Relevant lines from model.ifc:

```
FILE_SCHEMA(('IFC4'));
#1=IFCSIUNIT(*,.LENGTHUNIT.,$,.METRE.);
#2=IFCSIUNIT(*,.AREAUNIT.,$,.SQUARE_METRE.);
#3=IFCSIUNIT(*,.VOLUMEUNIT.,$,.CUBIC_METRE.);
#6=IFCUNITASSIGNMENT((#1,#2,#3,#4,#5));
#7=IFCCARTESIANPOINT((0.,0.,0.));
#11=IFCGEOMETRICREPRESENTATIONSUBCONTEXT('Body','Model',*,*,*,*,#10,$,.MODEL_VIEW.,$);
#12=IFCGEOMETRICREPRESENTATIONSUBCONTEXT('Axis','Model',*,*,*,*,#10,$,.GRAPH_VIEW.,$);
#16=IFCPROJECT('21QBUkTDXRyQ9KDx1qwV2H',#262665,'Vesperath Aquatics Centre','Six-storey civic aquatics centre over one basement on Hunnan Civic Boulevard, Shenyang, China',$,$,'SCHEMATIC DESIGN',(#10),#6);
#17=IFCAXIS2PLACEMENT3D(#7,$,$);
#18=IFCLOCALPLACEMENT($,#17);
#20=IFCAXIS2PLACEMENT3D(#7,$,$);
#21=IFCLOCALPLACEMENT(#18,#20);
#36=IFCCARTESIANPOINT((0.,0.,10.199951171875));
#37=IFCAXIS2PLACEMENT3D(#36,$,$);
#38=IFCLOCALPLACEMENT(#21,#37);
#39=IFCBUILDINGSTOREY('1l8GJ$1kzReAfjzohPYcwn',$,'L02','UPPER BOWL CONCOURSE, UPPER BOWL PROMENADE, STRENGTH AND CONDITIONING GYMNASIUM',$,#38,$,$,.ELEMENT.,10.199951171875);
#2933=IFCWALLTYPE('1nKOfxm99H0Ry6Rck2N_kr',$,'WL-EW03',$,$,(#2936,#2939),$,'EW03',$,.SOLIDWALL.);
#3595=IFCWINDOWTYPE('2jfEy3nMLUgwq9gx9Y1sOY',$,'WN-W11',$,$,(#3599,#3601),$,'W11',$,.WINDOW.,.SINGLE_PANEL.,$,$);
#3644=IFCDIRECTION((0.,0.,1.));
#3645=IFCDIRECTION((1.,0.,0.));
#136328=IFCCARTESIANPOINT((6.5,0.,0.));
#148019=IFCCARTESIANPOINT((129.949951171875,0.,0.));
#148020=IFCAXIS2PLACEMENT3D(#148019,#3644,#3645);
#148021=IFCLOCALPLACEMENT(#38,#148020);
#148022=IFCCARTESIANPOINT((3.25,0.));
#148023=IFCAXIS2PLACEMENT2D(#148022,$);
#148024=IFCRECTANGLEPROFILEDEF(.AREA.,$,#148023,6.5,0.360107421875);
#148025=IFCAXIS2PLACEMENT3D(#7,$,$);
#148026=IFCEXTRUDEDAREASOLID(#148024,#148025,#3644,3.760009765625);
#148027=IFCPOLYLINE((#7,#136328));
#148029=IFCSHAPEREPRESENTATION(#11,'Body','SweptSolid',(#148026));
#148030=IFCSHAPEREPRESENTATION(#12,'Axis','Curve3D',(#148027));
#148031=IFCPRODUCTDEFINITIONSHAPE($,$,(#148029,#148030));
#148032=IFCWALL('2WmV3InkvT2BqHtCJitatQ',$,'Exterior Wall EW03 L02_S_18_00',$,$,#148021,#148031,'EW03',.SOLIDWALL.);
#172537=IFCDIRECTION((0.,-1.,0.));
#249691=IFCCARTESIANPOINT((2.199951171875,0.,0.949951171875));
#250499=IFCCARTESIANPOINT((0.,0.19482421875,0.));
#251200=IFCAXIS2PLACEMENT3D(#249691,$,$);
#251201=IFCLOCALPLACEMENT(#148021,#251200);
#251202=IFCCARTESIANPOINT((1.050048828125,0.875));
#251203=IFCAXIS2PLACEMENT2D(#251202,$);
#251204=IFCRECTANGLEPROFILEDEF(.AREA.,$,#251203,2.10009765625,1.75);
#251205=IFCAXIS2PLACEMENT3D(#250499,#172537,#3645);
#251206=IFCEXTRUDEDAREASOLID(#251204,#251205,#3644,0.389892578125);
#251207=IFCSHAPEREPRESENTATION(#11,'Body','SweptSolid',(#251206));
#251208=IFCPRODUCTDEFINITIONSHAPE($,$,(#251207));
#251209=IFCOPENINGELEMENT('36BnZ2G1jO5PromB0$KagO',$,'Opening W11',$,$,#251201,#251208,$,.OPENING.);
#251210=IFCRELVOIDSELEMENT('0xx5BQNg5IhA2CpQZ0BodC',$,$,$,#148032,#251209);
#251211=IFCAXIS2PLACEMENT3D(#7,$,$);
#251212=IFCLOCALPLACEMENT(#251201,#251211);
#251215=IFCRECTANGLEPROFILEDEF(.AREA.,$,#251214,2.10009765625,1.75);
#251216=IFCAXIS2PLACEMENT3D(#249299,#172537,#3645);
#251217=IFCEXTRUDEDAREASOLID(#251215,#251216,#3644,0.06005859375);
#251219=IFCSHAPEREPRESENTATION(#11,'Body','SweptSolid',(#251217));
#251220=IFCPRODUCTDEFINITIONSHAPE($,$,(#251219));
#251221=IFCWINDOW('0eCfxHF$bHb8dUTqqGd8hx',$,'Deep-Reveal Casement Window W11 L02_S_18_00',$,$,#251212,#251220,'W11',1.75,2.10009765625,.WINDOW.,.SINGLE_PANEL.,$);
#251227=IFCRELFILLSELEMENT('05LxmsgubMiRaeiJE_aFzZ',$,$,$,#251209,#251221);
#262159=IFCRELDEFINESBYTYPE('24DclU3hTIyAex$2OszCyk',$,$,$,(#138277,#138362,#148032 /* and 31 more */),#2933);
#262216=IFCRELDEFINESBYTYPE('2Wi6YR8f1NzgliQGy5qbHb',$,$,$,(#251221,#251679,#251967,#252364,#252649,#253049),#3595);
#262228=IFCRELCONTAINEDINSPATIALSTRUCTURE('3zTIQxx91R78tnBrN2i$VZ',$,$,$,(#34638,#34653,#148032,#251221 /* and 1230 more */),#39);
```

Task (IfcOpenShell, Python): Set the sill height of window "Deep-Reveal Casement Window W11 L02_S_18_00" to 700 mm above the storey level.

```python
import numpy as np
import ifcopenshell
import ifcopenshell.api.geometry
import ifcopenshell.geom
import ifcopenshell.util.element
import ifcopenshell.util.placement
import ifcopenshell.util.shape
import ifcopenshell.util.unit

model = ifcopenshell.open("model.ifc")
unit_scale = ifcopenshell.util.unit.calculate_unit_scale(model)

window = model.by_guid("0eCfxHF$bHb8dUTqqGd8hx")
opening = window.FillsVoids[0].RelatingOpeningElement
storey = ifcopenshell.util.element.get_container(window, ifc_class="IfcBuildingStorey")
level = ifcopenshell.util.placement.get_local_placement(storey.ObjectPlacement)[2, 3]

# The opening's origin need not be at the sill, so measure its lowest point.
shape = ifcopenshell.geom.create_shape(ifcopenshell.geom.settings(), opening)
bottom = ifcopenshell.util.shape.get_shape_bottom_elevation(shape, shape.geometry) / unit_scale
dz = level + 0.7 / unit_scale - bottom

shift = np.array([0.0, 0.0, dz])
# The window is placed relative to its opening, so it follows when the opening moves.
matrix = ifcopenshell.util.placement.get_local_placement(opening.ObjectPlacement)
matrix[:3, 3] += shift
ifcopenshell.api.geometry.edit_object_placement(
    model, product=opening, matrix=matrix, is_si=False, should_transform_children=True
)

print(f"moved by {dz * unit_scale:+.3f} m")

model.write("model_updated.ifc")
```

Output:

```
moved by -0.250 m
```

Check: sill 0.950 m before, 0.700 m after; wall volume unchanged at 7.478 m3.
